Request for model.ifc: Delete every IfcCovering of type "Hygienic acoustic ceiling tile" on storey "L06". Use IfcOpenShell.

First a look at what the model holds.

```python
import ifcopenshell
import ifcopenshell.util.element

model = ifcopenshell.open("model.ifc")
print(model.schema)
storey = next(s for s in model.by_type("IfcBuildingStorey") if s.Name == "L06")
coverings = [e for e in ifcopenshell.util.element.get_decomposition(storey) if e.is_a("IfcCovering")]
seen = {}
for e in coverings:
    element_type = ifcopenshell.util.element.get_type(e)
    name = element_type.Name if element_type not in (None, e) else None
    seen[name] = seen.get(name, 0) + 1
for name, count in sorted(seen.items(), key=str):
    print(count, "x", name)
```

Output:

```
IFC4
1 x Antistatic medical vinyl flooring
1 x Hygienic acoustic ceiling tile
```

```python
import ifcopenshell
import ifcopenshell.api.root
import ifcopenshell.util.element

model = ifcopenshell.open("model.ifc")

storey = next(s for s in model.by_type("IfcBuildingStorey") if s.Name == "L06")
coverings = [e for e in ifcopenshell.util.element.get_decomposition(storey) if e.is_a("IfcCovering")]
targets = [e for e in coverings if (t := ifcopenshell.util.element.get_type(e)) not in (None, e) and t.Name == "Hygienic acoustic ceiling tile"]

for e in targets:
    ifcopenshell.api.root.remove_product(model, product=e)
print(len(targets), "removed")

model.write("model-out.ifc")
```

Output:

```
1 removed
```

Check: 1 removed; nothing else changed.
